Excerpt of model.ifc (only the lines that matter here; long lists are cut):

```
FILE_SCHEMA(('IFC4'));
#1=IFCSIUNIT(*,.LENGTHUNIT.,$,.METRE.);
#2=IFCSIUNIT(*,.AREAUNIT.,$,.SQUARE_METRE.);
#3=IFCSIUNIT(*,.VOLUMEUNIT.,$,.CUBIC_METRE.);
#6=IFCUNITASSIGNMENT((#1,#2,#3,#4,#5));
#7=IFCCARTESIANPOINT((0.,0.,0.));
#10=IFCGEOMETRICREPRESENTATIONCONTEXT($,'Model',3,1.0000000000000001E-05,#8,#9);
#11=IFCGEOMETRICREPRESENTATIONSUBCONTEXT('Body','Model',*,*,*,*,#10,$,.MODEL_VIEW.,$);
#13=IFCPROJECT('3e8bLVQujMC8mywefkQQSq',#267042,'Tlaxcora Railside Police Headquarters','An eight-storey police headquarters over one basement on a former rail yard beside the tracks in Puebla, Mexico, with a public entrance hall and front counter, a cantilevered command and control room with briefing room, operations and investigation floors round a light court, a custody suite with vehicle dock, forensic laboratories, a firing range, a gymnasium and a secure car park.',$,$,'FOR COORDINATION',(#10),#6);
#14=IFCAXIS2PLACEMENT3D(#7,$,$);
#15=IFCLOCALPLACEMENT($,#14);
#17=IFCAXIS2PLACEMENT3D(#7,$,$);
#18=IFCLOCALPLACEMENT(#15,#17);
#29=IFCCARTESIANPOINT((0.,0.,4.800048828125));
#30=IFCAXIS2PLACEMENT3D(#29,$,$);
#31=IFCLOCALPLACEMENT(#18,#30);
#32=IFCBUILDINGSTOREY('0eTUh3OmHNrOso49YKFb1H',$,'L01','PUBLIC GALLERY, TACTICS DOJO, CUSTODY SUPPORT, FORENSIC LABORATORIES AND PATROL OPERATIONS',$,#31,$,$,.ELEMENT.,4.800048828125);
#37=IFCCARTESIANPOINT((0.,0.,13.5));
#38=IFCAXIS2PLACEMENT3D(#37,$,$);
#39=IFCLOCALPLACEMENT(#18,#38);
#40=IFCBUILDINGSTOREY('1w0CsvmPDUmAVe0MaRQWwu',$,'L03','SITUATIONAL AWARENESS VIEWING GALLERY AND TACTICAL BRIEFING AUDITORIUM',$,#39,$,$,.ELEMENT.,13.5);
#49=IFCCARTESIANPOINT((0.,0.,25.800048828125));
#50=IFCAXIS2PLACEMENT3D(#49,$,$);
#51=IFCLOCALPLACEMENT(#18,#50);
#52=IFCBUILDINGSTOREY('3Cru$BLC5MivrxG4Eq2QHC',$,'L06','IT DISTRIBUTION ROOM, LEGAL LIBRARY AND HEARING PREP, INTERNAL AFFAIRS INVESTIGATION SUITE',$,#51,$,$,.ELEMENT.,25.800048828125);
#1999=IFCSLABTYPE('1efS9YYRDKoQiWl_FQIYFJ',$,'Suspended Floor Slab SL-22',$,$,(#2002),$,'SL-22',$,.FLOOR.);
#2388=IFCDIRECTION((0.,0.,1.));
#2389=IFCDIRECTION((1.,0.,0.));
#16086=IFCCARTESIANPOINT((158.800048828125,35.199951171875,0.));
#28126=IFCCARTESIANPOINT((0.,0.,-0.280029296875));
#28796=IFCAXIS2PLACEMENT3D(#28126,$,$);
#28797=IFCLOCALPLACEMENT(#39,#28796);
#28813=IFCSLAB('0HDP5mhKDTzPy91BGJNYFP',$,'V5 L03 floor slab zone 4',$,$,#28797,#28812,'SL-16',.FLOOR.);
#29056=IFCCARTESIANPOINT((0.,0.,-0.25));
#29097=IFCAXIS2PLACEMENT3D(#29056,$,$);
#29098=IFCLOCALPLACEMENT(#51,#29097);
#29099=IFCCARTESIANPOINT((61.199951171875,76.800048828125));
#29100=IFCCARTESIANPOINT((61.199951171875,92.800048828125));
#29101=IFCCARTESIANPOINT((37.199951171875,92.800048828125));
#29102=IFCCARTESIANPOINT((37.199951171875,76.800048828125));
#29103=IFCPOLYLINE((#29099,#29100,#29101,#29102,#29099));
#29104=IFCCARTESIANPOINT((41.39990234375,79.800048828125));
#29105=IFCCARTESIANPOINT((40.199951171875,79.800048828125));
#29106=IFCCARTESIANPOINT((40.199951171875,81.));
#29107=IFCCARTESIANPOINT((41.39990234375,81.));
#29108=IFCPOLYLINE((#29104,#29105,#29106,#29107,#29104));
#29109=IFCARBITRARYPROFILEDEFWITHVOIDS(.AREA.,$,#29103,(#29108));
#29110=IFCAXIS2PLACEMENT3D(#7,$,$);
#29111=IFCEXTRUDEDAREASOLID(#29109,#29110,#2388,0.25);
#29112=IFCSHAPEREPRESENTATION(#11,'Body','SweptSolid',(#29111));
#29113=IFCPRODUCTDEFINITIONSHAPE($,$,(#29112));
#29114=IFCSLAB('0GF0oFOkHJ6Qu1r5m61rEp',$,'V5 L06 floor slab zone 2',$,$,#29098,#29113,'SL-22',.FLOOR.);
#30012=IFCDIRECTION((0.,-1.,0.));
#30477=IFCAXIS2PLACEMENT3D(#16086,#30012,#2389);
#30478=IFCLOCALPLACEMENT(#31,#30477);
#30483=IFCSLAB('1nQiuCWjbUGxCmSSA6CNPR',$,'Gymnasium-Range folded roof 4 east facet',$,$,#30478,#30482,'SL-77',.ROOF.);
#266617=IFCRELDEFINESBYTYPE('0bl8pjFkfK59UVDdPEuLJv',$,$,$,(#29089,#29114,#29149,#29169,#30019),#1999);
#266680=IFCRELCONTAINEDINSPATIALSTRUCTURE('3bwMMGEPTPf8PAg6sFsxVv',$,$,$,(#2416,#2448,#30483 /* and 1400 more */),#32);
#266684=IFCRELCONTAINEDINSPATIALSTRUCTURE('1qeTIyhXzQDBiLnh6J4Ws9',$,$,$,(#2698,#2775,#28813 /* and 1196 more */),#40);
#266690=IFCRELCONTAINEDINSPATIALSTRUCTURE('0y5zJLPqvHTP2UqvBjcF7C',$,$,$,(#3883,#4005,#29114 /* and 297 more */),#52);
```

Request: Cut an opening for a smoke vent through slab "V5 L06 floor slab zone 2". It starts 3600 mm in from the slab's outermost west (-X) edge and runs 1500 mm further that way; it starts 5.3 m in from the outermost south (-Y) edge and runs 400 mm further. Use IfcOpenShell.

```python
import numpy as np
import ifcopenshell
import ifcopenshell.api.feature
import ifcopenshell.api.geometry
import ifcopenshell.api.root
import ifcopenshell.geom
import ifcopenshell.util.placement
import ifcopenshell.util.representation
import ifcopenshell.util.shape
import ifcopenshell.util.unit

model = ifcopenshell.open("model.ifc")
unit_scale = ifcopenshell.util.unit.calculate_unit_scale(model)
settings = ifcopenshell.geom.settings()


def volume(element):
    """Net volume in cubic metres, openings subtracted."""
    shape = ifcopenshell.geom.create_shape(settings, element)
    return ifcopenshell.util.shape.get_volume(shape.geometry)


slab = model.by_guid("0GF0oFOkHJ6Qu1r5m61rEp")
before = volume(slab)

# Extent in the slab's own axes, in metres. The edges named are its -X and -Y sides.
slab_shape = ifcopenshell.geom.create_shape(settings, slab)
vertices = ifcopenshell.util.shape.get_vertices(slab_shape.geometry)
x_min, y_min, bottom = vertices.min(axis=0)
top = vertices[:, 2].max()

opening = ifcopenshell.api.root.create_entity(model, ifc_class="IfcOpeningElement", name="Smoke vent opening", predefined_type="OPENING")
context = ifcopenshell.util.representation.get_context(model, "Model", "Body", "MODEL_VIEW")
width, depth = 1.5, 0.4
outline = [(0.0, 0.0), (width, 0.0), (width, depth), (0.0, depth), (0.0, 0.0)]
# Overshoot both faces by 50 mm so the cut is clean.
shape = ifcopenshell.api.geometry.add_slab_representation(
    model, context=context, depth=top - bottom + 0.1, polyline=outline
)
ifcopenshell.api.geometry.assign_representation(model, product=opening, representation=shape)

matrix = ifcopenshell.util.placement.get_local_placement(slab.ObjectPlacement)
matrix[:, 3] = matrix @ np.append(np.array([x_min + 3.6, y_min + 5.3, bottom - 0.05]) / unit_scale, 1.0)
ifcopenshell.api.geometry.edit_object_placement(model, product=opening, matrix=matrix, is_si=False)
ifcopenshell.api.feature.add_feature(model, feature=opening, element=slab)

after = volume(slab)

print(f"slab volume {before:.3f} -> {after:.3f} m3")

model.write("model_updated.ifc")
```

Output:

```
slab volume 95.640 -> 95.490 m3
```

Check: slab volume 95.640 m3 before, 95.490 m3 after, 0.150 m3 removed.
